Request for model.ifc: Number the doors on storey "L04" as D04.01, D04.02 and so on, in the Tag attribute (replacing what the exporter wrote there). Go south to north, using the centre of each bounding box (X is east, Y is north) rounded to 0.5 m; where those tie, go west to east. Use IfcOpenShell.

First a look at what the model holds.

```python
import ifcopenshell
import ifcopenshell.util.element
import ifcopenshell.util.placement

model = ifcopenshell.open("model.ifc")
print(model.schema)
storey = next(s for s in model.by_type("IfcBuildingStorey") if s.Name == "L04")
doors = [e for e in ifcopenshell.util.element.get_decomposition(storey) if e.is_a("IfcDoor")]
for e in sorted(doors, key=lambda e: e.id()):
    origin = ifcopenshell.util.placement.get_local_placement(e.ObjectPlacement)[:3, 3]
    print(e.id(), e.Tag, e.Name, origin.round(2) + 0.0, sep=" | ")
```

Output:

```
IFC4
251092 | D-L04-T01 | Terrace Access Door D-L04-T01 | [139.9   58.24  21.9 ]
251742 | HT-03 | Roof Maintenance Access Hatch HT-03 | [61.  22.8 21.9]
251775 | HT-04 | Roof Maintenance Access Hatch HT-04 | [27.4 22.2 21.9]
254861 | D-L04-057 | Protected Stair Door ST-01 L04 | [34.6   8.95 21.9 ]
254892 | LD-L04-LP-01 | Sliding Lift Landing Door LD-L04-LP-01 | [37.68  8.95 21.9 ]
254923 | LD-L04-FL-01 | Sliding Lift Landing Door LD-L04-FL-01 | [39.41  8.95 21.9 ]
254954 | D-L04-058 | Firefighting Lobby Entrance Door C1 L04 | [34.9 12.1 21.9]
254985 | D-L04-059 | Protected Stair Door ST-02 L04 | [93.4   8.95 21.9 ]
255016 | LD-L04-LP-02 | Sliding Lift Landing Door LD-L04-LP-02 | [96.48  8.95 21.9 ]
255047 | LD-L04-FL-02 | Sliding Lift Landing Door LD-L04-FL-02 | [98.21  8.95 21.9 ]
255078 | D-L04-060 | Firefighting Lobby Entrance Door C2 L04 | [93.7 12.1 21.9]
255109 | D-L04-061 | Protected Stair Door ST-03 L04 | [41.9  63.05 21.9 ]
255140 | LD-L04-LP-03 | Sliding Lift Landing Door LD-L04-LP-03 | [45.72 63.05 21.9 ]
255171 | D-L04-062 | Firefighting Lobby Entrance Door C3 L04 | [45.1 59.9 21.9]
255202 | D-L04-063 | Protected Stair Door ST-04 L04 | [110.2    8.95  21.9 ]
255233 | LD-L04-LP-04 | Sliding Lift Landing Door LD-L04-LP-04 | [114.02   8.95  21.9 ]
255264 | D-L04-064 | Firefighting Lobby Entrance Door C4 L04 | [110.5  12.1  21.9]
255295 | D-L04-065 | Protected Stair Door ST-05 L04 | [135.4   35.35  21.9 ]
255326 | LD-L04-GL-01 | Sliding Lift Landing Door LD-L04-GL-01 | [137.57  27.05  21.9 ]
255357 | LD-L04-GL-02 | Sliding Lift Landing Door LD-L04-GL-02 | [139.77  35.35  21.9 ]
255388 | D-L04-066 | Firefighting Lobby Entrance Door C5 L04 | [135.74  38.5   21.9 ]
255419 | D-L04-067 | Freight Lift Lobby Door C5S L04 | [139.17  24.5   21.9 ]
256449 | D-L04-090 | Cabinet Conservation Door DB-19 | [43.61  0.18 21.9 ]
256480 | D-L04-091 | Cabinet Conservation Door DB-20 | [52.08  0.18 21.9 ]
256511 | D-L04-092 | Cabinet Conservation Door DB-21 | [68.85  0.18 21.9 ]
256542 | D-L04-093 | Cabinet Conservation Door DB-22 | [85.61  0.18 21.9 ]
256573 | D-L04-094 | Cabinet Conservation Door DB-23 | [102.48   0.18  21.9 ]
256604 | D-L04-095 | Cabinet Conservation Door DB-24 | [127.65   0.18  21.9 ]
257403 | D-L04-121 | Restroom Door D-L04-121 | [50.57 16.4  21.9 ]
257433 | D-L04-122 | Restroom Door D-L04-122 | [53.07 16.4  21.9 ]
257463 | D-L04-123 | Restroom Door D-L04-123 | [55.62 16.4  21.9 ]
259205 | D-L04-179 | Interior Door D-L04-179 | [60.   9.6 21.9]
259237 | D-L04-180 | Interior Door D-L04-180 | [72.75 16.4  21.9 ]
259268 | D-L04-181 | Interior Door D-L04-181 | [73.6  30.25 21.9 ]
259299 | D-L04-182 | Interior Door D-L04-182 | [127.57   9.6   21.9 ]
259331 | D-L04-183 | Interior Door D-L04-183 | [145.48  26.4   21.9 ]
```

```python
import ifcopenshell
import ifcopenshell.geom
import ifcopenshell.util.element
import ifcopenshell.util.shape

model = ifcopenshell.open("model.ifc")
settings = ifcopenshell.geom.settings()
settings.set("use-world-coords", True)


def centre(element):
    shape = ifcopenshell.geom.create_shape(settings, element)
    return ifcopenshell.util.shape.get_bbox_centroid(shape.geometry)


storey = next(s for s in model.by_type("IfcBuildingStorey") if s.Name == "L04")
doors = [e for e in ifcopenshell.util.element.get_decomposition(storey) if e.is_a("IfcDoor")]

# Insertion points can sit at a corner or the storey origin, so sort by the geometry (in metres).
centres = {e: centre(e) for e in doors}
doors.sort(key=lambda e: (round(centres[e][1] / 0.5), centres[e][0]))

for i, e in enumerate(doors, start=1):
    number = f"D04.{i:02d}"
    e.Tag = number
    print(e.id(), number)

model.write("model_updated.ifc")
```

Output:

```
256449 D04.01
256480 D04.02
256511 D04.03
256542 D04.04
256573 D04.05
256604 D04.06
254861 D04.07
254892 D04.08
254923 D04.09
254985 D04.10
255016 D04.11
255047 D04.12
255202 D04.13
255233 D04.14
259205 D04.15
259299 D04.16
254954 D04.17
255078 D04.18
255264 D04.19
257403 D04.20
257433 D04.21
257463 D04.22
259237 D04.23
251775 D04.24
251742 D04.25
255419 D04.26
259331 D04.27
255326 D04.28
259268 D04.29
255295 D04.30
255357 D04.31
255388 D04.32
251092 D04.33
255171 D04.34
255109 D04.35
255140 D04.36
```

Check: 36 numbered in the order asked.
